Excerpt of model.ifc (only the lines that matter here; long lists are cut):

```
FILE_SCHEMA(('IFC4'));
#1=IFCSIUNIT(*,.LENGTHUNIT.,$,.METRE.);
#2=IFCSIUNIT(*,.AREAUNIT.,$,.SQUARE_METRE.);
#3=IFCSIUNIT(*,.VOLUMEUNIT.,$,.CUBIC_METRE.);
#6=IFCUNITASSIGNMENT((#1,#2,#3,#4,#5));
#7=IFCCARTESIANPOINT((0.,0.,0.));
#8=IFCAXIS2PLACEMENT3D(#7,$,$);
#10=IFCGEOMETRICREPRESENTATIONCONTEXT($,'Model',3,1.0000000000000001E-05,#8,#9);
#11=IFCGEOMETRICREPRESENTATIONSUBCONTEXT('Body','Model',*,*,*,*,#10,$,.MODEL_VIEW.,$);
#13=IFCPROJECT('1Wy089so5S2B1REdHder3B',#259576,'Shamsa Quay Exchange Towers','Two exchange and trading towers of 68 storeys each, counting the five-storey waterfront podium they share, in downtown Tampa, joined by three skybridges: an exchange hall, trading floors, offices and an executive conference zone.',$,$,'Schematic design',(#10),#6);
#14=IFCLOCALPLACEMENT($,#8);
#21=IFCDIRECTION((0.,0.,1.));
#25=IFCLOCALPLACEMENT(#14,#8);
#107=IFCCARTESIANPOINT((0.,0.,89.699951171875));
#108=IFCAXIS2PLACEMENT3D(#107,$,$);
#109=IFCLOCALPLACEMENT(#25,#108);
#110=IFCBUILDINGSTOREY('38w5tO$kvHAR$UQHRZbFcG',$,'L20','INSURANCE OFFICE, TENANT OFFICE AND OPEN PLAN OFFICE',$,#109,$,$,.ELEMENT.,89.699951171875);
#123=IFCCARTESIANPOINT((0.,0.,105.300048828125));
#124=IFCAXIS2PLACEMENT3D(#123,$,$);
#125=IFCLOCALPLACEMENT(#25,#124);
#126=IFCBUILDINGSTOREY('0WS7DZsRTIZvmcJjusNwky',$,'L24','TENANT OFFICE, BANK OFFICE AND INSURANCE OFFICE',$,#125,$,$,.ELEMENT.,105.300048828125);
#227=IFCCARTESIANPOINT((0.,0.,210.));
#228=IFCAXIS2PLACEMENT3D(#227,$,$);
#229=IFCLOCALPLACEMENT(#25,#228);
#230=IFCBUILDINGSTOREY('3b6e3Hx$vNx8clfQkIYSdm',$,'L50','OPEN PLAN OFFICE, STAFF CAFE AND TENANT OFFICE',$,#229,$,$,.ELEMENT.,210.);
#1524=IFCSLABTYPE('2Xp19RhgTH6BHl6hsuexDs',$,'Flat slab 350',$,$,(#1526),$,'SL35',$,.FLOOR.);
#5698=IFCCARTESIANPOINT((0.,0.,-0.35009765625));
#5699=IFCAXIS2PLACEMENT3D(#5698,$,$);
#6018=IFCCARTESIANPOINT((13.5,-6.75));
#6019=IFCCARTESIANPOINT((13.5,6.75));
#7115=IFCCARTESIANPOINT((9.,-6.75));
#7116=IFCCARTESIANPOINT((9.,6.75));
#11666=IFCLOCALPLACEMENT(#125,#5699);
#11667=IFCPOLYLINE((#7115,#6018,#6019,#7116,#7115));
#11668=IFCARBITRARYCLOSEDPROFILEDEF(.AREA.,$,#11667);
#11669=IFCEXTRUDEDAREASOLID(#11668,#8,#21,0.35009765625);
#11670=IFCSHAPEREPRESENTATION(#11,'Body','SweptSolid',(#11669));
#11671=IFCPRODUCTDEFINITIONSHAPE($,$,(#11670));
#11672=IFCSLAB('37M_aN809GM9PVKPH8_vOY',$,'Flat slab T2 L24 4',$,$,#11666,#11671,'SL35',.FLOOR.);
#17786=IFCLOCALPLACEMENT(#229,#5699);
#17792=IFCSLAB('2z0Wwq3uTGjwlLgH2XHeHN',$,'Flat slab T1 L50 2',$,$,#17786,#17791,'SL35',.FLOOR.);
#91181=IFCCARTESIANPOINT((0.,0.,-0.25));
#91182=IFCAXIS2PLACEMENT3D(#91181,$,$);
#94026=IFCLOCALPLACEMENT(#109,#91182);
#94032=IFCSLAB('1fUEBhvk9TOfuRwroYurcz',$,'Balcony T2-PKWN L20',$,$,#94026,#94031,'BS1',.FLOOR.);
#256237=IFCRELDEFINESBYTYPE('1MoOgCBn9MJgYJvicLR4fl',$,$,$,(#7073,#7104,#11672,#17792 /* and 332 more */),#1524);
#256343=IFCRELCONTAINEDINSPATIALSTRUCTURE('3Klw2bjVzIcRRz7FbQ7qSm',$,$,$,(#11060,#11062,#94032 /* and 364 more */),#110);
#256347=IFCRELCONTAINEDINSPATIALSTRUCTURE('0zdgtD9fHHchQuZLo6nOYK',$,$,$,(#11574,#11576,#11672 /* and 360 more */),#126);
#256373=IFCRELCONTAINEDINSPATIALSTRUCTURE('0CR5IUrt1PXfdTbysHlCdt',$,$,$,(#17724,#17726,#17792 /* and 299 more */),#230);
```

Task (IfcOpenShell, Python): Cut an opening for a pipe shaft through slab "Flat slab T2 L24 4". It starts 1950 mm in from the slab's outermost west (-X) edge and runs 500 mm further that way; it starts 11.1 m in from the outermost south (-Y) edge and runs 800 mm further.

```python
import numpy as np
import ifcopenshell
import ifcopenshell.api.feature
import ifcopenshell.api.geometry
import ifcopenshell.api.root
import ifcopenshell.geom
import ifcopenshell.util.placement
import ifcopenshell.util.representation
import ifcopenshell.util.shape
import ifcopenshell.util.unit

model = ifcopenshell.open("model.ifc")
unit_scale = ifcopenshell.util.unit.calculate_unit_scale(model)
settings = ifcopenshell.geom.settings()


def volume(element):
    """Net volume in cubic metres, openings subtracted."""
    shape = ifcopenshell.geom.create_shape(settings, element)
    return ifcopenshell.util.shape.get_volume(shape.geometry)


slab = model.by_id(11672)
before = volume(slab)

# Extent in the slab's own axes, in metres. The edges named are its -X and -Y sides.
slab_shape = ifcopenshell.geom.create_shape(settings, slab)
vertices = ifcopenshell.util.shape.get_vertices(slab_shape.geometry)
x_min, y_min, bottom = vertices.min(axis=0)
top = vertices[:, 2].max()

opening = ifcopenshell.api.root.create_entity(model, ifc_class="IfcOpeningElement", name="Pipe shaft opening", predefined_type="OPENING")
context = ifcopenshell.util.representation.get_context(model, "Model", "Body", "MODEL_VIEW")
width, depth = 0.5, 0.8
outline = [(0.0, 0.0), (width, 0.0), (width, depth), (0.0, depth), (0.0, 0.0)]
# Overshoot both faces by 50 mm so the cut is clean.
shape = ifcopenshell.api.geometry.add_slab_representation(
    model, context=context, depth=top - bottom + 0.1, polyline=outline
)
ifcopenshell.api.geometry.assign_representation(model, product=opening, representation=shape)

matrix = ifcopenshell.util.placement.get_local_placement(slab.ObjectPlacement)
matrix[:, 3] = matrix @ np.append(np.array([x_min + 1.95, y_min + 11.1, bottom - 0.05]) / unit_scale, 1.0)
ifcopenshell.api.geometry.edit_object_placement(model, product=opening, matrix=matrix, is_si=False)
ifcopenshell.api.feature.add_feature(model, feature=opening, element=slab)

after = volume(slab)

print(f"slab volume {before:.3f} -> {after:.3f} m3")

model.write("model_updated.ifc")
```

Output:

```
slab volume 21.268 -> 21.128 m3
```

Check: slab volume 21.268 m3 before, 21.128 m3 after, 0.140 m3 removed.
